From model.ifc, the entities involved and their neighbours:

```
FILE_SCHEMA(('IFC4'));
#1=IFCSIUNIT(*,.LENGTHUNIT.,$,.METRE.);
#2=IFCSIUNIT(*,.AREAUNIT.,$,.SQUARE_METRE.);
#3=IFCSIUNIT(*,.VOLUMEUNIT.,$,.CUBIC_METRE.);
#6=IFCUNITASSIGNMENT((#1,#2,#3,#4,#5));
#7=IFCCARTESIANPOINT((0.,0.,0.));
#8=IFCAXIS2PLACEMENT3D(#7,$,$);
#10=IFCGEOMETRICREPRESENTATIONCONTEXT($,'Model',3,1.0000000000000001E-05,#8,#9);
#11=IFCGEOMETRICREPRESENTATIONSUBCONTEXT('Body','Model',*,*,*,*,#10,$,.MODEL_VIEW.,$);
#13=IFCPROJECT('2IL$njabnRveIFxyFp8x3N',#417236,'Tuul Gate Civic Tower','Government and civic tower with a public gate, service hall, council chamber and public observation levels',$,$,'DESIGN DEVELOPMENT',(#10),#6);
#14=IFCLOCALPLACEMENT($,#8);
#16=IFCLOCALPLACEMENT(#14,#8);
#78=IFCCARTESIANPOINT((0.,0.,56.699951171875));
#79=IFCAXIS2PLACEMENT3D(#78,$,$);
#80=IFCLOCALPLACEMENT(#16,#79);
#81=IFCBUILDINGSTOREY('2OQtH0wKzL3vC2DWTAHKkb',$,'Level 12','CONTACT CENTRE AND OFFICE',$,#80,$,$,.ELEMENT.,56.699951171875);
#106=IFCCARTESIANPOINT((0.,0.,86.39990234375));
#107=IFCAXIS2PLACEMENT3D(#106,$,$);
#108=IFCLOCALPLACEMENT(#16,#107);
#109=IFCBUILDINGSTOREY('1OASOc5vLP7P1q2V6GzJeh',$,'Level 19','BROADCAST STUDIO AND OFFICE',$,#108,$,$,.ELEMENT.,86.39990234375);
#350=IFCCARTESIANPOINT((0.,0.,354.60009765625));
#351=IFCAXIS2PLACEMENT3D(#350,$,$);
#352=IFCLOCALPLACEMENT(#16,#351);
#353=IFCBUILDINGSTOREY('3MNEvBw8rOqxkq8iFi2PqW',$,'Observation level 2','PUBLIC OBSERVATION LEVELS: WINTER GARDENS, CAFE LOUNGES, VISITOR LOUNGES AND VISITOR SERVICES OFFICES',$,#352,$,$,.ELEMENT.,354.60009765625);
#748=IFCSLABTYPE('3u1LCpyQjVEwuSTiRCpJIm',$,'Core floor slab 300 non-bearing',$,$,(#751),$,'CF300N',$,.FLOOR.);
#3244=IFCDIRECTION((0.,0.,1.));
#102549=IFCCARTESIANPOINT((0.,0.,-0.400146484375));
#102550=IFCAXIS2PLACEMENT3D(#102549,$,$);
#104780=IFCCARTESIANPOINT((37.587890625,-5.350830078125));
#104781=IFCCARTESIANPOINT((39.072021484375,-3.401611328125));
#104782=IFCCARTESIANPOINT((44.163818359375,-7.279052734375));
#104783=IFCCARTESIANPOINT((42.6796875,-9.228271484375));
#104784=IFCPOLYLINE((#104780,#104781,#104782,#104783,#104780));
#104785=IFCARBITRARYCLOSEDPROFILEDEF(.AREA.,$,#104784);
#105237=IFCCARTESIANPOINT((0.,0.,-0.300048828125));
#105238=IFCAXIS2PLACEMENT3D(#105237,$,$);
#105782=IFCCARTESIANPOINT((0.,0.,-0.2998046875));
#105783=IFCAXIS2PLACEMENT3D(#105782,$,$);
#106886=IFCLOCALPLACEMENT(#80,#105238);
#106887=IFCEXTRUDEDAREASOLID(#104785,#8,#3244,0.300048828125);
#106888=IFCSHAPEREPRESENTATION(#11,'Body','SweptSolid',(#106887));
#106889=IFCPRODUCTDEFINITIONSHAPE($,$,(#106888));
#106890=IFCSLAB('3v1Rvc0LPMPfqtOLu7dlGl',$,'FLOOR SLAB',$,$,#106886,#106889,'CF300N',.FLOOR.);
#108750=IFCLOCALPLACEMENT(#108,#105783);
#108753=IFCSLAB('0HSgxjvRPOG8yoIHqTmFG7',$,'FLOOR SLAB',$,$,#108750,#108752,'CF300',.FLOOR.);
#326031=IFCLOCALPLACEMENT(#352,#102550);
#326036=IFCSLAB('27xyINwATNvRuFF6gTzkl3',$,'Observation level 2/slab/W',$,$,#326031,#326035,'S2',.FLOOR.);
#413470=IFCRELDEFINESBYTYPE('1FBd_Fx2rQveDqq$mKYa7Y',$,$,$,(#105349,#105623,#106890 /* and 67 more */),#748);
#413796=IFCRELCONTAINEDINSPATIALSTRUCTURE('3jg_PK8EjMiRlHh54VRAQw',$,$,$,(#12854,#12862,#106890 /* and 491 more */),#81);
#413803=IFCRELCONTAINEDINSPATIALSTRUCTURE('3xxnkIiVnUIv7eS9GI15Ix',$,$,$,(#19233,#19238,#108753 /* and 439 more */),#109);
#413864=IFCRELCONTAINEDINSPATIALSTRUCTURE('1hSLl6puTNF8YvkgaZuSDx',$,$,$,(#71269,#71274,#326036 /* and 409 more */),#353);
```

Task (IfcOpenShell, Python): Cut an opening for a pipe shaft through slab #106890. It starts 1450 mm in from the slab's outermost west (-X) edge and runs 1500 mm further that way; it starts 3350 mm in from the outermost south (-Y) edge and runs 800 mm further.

```python
import numpy as np
import ifcopenshell
import ifcopenshell.api.feature
import ifcopenshell.api.geometry
import ifcopenshell.api.root
import ifcopenshell.geom
import ifcopenshell.util.placement
import ifcopenshell.util.representation
import ifcopenshell.util.shape
import ifcopenshell.util.unit

model = ifcopenshell.open("model.ifc")
unit_scale = ifcopenshell.util.unit.calculate_unit_scale(model)
settings = ifcopenshell.geom.settings()


def volume(element):
    """Net volume in cubic metres, openings subtracted."""
    shape = ifcopenshell.geom.create_shape(settings, element)
    return ifcopenshell.util.shape.get_volume(shape.geometry)


slab = model.by_id(106890)
before = volume(slab)

# Extent in the slab's own axes, in metres. The edges named are its -X and -Y sides.
slab_shape = ifcopenshell.geom.create_shape(settings, slab)
vertices = ifcopenshell.util.shape.get_vertices(slab_shape.geometry)
x_min, y_min, bottom = vertices.min(axis=0)
top = vertices[:, 2].max()

opening = ifcopenshell.api.root.create_entity(model, ifc_class="IfcOpeningElement", name="Pipe shaft opening", predefined_type="OPENING")
context = ifcopenshell.util.representation.get_context(model, "Model", "Body", "MODEL_VIEW")
width, depth = 1.5, 0.8
outline = [(0.0, 0.0), (width, 0.0), (width, depth), (0.0, depth), (0.0, 0.0)]
# Overshoot both faces by 50 mm so the cut is clean.
shape = ifcopenshell.api.geometry.add_slab_representation(
    model, context=context, depth=top - bottom + 0.1, polyline=outline
)
ifcopenshell.api.geometry.assign_representation(model, product=opening, representation=shape)

matrix = ifcopenshell.util.placement.get_local_placement(slab.ObjectPlacement)
matrix[:, 3] = matrix @ np.append(np.array([x_min + 1.45, y_min + 3.35, bottom - 0.05]) / unit_scale, 1.0)
ifcopenshell.api.geometry.edit_object_placement(model, product=opening, matrix=matrix, is_si=False)
ifcopenshell.api.feature.add_feature(model, feature=opening, element=slab)

after = volume(slab)

print(f"slab volume {before:.3f} -> {after:.3f} m3")

model.write("model_edited.ifc")
```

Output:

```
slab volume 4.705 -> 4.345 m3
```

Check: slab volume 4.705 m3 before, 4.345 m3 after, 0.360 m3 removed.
